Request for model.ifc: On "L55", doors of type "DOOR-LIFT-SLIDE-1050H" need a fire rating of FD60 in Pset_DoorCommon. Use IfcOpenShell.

First a look at what the model holds.

```python
import ifcopenshell
import ifcopenshell.util.element

model = ifcopenshell.open("model.ifc")
print(model.schema)
storey = next(s for s in model.by_type("IfcBuildingStorey") if s.Name == "L55")
doors = [e for e in ifcopenshell.util.element.get_decomposition(storey) if e.is_a("IfcDoor")]
seen = {}
for e in doors:
    element_type = ifcopenshell.util.element.get_type(e)
    key = (element_type.Name if element_type != e and element_type else None, ifcopenshell.util.element.get_pset(e, "Pset_DoorCommon", "FireRating"))
    seen[key] = seen.get(key, 0) + 1
for (name, value), count in sorted(seen.items(), key=str):
    print(count, "x", name, "|", value)
```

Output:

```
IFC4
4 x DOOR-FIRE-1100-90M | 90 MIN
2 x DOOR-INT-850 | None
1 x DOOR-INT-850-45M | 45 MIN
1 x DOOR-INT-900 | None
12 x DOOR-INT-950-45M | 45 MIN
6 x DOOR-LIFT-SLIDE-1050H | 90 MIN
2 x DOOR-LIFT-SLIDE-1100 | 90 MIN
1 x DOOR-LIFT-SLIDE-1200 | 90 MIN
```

```python
import ifcopenshell
import ifcopenshell.api.pset
import ifcopenshell.util.element

model = ifcopenshell.open("model.ifc")

storey = next(s for s in model.by_type("IfcBuildingStorey") if s.Name == "L55")
doors = [e for e in ifcopenshell.util.element.get_decomposition(storey) if e.is_a("IfcDoor")]

count = 0
for e in doors:
    element_type = ifcopenshell.util.element.get_type(e)
    if element_type in (None, e) or element_type.Name != "DOOR-LIFT-SLIDE-1050H":
        continue
    found = ifcopenshell.util.element.get_pset(e, "Pset_DoorCommon", should_inherit=False)
    if found:
        pset = model.by_id(found["id"])
        if len(ifcopenshell.util.element.get_elements_by_pset(pset)) > 1:
            pset = ifcopenshell.api.pset.unshare_pset(model, products=[e], pset=pset)[0]
    else:
        pset = ifcopenshell.api.pset.add_pset(model, product=e, name="Pset_DoorCommon")
    ifcopenshell.api.pset.edit_pset(model, pset=pset, properties={"FireRating": "FD60"})
    count += 1

print(count, "doors updated")

model.write("model_v2.ifc")
```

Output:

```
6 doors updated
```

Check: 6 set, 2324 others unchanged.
